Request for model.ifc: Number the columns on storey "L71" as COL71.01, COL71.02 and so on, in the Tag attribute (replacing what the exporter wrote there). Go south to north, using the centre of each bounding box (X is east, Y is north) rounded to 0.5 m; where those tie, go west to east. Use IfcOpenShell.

First a look at what the model holds.

```python
import ifcopenshell
import ifcopenshell.util.element
import ifcopenshell.util.placement

model = ifcopenshell.open("model.ifc")
print(model.schema)
storey = next(s for s in model.by_type("IfcBuildingStorey") if s.Name == "L71")
columns = [e for e in ifcopenshell.util.element.get_decomposition(storey) if e.is_a("IfcColumn")]
for e in sorted(columns, key=lambda e: e.id()):
    origin = ifcopenshell.util.placement.get_local_placement(e.ObjectPlacement)[:3, 3]
    print(e.id(), e.Tag, e.Name, origin.round(2) + 0.0, sep=" | ")
```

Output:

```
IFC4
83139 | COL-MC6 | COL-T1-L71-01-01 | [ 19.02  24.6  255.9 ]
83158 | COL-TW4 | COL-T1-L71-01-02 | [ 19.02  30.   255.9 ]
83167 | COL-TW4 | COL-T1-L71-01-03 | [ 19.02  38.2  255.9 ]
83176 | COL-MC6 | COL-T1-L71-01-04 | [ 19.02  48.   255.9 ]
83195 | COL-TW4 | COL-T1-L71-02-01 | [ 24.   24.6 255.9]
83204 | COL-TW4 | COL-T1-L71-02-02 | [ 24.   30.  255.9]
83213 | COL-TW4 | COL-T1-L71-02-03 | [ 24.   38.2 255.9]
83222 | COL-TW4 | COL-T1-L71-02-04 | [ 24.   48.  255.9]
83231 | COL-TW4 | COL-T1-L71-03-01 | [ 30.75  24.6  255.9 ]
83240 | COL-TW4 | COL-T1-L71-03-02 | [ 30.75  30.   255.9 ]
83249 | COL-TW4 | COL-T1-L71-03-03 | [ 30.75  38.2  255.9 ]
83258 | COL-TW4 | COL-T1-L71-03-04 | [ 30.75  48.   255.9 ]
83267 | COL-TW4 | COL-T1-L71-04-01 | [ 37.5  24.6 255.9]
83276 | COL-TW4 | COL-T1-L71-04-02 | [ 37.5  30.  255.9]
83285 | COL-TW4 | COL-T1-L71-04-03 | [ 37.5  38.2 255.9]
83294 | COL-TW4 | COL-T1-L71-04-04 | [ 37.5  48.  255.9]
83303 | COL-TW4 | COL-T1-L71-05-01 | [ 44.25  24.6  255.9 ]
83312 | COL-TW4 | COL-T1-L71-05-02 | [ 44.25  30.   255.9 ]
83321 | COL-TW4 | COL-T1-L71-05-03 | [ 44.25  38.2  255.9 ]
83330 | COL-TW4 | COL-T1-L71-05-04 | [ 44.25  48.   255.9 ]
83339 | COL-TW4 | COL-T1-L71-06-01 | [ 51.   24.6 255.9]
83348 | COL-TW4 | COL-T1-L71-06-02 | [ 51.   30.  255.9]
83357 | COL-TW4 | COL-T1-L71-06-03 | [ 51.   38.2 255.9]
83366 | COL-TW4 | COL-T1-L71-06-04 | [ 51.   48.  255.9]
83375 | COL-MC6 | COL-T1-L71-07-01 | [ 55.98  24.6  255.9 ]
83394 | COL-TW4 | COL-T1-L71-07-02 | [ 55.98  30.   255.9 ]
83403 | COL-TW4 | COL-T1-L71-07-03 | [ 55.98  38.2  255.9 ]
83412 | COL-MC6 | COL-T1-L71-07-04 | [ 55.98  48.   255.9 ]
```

```python
import ifcopenshell
import ifcopenshell.geom
import ifcopenshell.util.element
import ifcopenshell.util.shape

model = ifcopenshell.open("model.ifc")
settings = ifcopenshell.geom.settings()
settings.set("use-world-coords", True)


def centre(element):
    shape = ifcopenshell.geom.create_shape(settings, element)
    return ifcopenshell.util.shape.get_bbox_centroid(shape.geometry)


storey = next(s for s in model.by_type("IfcBuildingStorey") if s.Name == "L71")
columns = [e for e in ifcopenshell.util.element.get_decomposition(storey) if e.is_a("IfcColumn")]

# Insertion points can sit at a corner or the storey origin, so sort by the geometry (in metres).
centres = {e: centre(e) for e in columns}
columns.sort(key=lambda e: (round(centres[e][1] / 0.5), centres[e][0]))

for i, e in enumerate(columns, start=1):
    number = f"COL71.{i:02d}"
    e.Tag = number
    print(e.id(), number)

model.write("model_updated.ifc")
```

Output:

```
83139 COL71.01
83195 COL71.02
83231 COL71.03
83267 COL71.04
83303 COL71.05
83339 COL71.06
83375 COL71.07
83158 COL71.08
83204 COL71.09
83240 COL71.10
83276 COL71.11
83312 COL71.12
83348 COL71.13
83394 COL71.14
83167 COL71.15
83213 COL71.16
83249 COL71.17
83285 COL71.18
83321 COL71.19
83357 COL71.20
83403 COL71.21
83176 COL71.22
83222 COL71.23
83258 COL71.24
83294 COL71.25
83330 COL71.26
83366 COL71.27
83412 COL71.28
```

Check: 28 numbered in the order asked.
